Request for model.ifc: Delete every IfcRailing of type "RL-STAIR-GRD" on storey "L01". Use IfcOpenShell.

First a look at what the model holds.

```python
import ifcopenshell
import ifcopenshell.util.element

model = ifcopenshell.open("model.ifc")
print(model.schema)
storey = next(s for s in model.by_type("IfcBuildingStorey") if s.Name == "L01")
railings = [e for e in ifcopenshell.util.element.get_decomposition(storey) if e.is_a("IfcRailing")]
seen = {}
for e in railings:
    element_type = ifcopenshell.util.element.get_type(e)
    name = element_type.Name if element_type not in (None, e) else None
    seen[name] = seen.get(name, 0) + 1
for name, count in sorted(seen.items(), key=str):
    print(count, "x", name)
```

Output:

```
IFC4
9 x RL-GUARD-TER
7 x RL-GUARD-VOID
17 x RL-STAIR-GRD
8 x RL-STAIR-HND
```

```python
import ifcopenshell
import ifcopenshell.api.root
import ifcopenshell.util.element

model = ifcopenshell.open("model.ifc")

storey = next(s for s in model.by_type("IfcBuildingStorey") if s.Name == "L01")
railings = [e for e in ifcopenshell.util.element.get_decomposition(storey) if e.is_a("IfcRailing")]
targets = [e for e in railings if (t := ifcopenshell.util.element.get_type(e)) not in (None, e) and t.Name == "RL-STAIR-GRD"]

for e in targets:
    ifcopenshell.api.root.remove_product(model, product=e)
print(len(targets), "removed")

model.write("model_v2.ifc")
```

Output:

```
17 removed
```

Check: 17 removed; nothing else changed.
